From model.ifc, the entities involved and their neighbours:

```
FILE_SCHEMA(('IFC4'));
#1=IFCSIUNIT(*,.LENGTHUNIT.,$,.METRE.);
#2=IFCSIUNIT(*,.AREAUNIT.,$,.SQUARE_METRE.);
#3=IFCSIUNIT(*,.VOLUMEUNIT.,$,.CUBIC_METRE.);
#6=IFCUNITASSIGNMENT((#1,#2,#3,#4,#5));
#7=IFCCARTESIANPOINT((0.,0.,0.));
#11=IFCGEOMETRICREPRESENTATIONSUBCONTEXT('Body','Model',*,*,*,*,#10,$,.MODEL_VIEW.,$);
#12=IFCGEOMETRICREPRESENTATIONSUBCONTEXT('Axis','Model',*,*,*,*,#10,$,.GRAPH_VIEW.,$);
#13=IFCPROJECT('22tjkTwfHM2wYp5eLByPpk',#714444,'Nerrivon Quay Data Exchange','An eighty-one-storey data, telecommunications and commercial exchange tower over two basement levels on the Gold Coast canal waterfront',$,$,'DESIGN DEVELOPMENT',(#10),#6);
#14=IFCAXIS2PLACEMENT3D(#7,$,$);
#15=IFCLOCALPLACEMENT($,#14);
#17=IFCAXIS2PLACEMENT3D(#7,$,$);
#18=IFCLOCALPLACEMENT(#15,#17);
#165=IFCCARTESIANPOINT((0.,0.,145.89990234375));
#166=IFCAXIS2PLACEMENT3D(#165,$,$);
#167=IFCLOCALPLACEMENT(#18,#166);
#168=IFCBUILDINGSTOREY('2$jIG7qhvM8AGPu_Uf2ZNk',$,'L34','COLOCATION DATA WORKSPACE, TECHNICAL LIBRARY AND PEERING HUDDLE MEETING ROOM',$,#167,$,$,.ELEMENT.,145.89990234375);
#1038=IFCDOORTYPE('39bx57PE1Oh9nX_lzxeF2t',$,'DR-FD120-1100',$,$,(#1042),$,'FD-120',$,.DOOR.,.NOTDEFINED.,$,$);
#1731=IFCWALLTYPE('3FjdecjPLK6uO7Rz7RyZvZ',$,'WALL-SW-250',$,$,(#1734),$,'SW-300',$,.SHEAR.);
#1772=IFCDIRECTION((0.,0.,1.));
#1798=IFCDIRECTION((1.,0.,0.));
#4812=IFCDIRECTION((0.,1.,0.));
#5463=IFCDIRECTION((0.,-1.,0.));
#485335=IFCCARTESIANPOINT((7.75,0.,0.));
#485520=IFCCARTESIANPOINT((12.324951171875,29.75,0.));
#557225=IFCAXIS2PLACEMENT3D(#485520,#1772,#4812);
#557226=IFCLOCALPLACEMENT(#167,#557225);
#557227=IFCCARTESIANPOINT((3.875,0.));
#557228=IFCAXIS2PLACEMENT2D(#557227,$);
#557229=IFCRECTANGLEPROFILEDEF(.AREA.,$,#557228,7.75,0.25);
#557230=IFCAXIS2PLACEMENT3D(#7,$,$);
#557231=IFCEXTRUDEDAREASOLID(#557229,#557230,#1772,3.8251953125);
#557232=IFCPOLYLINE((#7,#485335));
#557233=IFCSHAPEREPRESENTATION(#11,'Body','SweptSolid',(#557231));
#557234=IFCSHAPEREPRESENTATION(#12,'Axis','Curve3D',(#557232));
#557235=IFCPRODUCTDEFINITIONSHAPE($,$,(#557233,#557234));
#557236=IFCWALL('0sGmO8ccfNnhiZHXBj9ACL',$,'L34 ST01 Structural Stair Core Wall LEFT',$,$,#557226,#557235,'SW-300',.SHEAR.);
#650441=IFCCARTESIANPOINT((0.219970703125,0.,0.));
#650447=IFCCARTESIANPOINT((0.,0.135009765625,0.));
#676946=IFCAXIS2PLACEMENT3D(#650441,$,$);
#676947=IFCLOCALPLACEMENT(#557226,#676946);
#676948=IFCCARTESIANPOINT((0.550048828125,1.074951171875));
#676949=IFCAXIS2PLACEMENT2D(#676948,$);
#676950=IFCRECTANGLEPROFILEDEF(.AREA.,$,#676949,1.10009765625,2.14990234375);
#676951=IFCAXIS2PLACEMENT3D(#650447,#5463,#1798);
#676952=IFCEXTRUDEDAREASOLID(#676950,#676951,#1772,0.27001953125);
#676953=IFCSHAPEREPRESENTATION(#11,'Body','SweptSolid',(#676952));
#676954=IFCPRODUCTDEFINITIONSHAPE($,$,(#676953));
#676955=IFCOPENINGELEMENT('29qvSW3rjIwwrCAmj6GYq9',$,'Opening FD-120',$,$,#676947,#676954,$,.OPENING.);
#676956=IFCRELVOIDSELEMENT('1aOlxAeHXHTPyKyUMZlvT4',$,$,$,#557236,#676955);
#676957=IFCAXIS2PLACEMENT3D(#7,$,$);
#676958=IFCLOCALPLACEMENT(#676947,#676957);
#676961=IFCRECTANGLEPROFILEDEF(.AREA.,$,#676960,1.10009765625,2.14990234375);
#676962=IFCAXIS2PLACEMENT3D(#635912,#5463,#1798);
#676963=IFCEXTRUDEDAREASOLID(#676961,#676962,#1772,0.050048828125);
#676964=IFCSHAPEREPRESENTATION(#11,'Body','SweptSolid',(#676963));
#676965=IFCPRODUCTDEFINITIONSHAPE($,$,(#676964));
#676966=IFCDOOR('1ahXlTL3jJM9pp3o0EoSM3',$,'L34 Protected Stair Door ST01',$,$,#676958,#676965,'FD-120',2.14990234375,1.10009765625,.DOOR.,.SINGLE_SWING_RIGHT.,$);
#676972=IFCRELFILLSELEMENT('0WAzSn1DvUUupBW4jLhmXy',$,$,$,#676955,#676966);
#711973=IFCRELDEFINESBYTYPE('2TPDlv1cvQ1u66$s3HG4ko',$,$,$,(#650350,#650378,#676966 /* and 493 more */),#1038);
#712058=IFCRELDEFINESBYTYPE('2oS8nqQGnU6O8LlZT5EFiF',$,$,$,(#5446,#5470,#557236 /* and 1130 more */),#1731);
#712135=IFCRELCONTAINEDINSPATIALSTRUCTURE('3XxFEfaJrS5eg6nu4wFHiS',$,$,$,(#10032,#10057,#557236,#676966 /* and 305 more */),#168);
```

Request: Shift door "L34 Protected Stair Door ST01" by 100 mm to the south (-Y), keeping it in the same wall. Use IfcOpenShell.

```python
import ifcopenshell
import ifcopenshell.api.geometry
import ifcopenshell.util.placement
import ifcopenshell.util.unit

model = ifcopenshell.open("model.ifc")
unit_scale = ifcopenshell.util.unit.calculate_unit_scale(model)

door = model.by_guid("1ahXlTL3jJM9pp3o0EoSM3")
opening = door.FillsVoids[0].RelatingOpeningElement
wall = opening.VoidsElements[0].RelatingBuildingElement

wall_matrix = ifcopenshell.util.placement.get_local_placement(wall.ObjectPlacement)
shift = wall_matrix[:3, 0] * -0.1 / unit_scale
before = ifcopenshell.util.placement.get_local_placement(door.ObjectPlacement)[:3, 3].copy()

# The door is placed relative to its opening, so it follows when the opening moves.
matrix = ifcopenshell.util.placement.get_local_placement(opening.ObjectPlacement)
matrix[:3, 3] += shift
ifcopenshell.api.geometry.edit_object_placement(
    model, product=opening, matrix=matrix, is_si=False, should_transform_children=True
)

after = ifcopenshell.util.placement.get_local_placement(door.ObjectPlacement)[:3, 3]
print("door moved by", (after - before).round(3) + 0.0)

model.write("model_rev.ifc")
```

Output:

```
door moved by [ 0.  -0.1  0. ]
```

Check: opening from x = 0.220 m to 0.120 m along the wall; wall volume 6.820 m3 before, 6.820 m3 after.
